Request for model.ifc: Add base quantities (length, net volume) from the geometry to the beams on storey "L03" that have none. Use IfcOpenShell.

First a look at what the model holds.

```python
import ifcopenshell
import ifcopenshell.util.element
import ifcopenshell.util.unit

model = ifcopenshell.open("model.ifc")
print(model.schema)
for unit_type in ("LENGTHUNIT", "AREAUNIT", "VOLUMEUNIT"):
    print(unit_type, ifcopenshell.util.unit.calculate_unit_scale(model, unit_type))
storey = next(s for s in model.by_type("IfcBuildingStorey") if s.Name == "L03")
beams = [e for e in ifcopenshell.util.element.get_decomposition(storey) if e.is_a("IfcBeam")]
for e in sorted(beams, key=lambda e: e.id()):
    print(e.id(), e.is_a(), e.Name, list(ifcopenshell.util.element.get_psets(e, qtos_only=True)), sep=" | ")
```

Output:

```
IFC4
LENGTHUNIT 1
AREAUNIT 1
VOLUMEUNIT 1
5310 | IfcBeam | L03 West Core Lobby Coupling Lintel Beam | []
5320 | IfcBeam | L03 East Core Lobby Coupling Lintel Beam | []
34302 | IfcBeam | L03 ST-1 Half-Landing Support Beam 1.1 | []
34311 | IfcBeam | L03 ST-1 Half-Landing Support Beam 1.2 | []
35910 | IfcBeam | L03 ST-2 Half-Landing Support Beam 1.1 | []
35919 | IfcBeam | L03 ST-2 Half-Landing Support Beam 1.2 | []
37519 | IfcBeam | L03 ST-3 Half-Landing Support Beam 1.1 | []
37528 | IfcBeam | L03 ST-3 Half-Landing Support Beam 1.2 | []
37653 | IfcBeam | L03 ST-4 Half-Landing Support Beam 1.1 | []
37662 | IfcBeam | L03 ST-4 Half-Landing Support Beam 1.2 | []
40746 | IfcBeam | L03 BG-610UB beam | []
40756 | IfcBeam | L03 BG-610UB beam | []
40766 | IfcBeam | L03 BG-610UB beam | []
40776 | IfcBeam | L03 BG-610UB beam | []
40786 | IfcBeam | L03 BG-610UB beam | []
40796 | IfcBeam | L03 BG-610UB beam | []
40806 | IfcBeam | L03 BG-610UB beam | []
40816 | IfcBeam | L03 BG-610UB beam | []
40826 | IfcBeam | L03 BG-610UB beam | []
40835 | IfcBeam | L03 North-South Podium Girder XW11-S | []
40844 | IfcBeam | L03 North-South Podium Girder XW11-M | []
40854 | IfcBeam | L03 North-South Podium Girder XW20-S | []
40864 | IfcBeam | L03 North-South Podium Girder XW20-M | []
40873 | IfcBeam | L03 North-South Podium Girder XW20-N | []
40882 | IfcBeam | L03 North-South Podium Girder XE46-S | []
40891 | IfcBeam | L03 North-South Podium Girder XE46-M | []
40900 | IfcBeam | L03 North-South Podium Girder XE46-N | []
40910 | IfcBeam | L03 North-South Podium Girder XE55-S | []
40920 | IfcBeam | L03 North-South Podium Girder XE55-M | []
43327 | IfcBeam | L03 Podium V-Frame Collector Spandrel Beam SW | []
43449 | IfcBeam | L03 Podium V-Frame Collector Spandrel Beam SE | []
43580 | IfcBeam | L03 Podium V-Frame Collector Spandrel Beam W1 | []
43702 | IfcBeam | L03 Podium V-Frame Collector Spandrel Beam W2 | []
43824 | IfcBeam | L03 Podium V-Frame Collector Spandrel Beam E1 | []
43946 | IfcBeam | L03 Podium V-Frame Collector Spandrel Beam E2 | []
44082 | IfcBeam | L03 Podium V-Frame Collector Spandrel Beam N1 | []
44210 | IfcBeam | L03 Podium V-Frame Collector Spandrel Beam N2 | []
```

```python
import ifcopenshell
import ifcopenshell.api.pset
import ifcopenshell.geom
import ifcopenshell.util.element
import ifcopenshell.util.shape
import ifcopenshell.util.unit

model = ifcopenshell.open("model.ifc")
unit_scale = ifcopenshell.util.unit.calculate_unit_scale(model)
volume_scale = ifcopenshell.util.unit.calculate_unit_scale(model, "VOLUMEUNIT")
settings = ifcopenshell.geom.settings()

storey = next(s for s in model.by_type("IfcBuildingStorey") if s.Name == "L03")
beams = [e for e in ifcopenshell.util.element.get_decomposition(storey) if e.is_a("IfcBeam")]

for e in sorted(beams, key=lambda e: e.id()):
    if ifcopenshell.util.element.get_psets(e, qtos_only=True, should_inherit=False):
        continue
    # Geometry comes back in metres, in the element's own axes.
    shape = ifcopenshell.geom.create_shape(settings, e)
    values = {
        "Length": ifcopenshell.util.shape.get_max_xyz(shape.geometry) / unit_scale,
        "NetVolume": ifcopenshell.util.shape.get_volume(shape.geometry) / volume_scale,
    }
    qto = ifcopenshell.api.pset.add_qto(model, product=e, name="Qto_BeamBaseQuantities")
    ifcopenshell.api.pset.edit_qto(model, qto=qto, properties=values)
    print(e.id(), {k: round(v, 3) for k, v in values.items()})

model.write("model_edited.ifc")
```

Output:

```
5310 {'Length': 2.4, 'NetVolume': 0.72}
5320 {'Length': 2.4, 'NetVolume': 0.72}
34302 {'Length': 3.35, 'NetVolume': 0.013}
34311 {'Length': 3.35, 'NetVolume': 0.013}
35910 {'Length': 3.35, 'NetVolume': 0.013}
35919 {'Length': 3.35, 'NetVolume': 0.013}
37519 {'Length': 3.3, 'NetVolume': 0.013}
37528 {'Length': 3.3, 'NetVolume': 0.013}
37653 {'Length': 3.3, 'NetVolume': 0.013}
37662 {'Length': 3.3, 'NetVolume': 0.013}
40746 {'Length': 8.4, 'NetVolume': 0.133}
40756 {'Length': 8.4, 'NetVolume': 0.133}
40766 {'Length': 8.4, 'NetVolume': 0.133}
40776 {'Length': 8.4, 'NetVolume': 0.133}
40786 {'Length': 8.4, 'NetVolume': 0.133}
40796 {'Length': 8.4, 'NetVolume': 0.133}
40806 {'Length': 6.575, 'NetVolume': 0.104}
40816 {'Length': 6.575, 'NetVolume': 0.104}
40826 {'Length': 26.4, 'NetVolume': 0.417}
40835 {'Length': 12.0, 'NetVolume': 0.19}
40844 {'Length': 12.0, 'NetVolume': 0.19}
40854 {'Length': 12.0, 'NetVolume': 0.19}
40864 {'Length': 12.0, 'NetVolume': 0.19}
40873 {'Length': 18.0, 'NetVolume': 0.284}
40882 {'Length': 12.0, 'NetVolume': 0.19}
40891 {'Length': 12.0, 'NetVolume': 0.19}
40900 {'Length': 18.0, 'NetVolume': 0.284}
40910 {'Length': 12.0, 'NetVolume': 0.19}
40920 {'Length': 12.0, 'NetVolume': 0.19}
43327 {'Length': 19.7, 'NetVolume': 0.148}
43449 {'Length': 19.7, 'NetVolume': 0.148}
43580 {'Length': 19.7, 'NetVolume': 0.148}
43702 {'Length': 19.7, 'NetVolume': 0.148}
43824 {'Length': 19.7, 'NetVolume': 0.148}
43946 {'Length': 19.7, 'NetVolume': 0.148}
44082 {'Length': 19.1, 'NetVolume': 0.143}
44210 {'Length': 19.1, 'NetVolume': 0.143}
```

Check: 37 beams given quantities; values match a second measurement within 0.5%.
